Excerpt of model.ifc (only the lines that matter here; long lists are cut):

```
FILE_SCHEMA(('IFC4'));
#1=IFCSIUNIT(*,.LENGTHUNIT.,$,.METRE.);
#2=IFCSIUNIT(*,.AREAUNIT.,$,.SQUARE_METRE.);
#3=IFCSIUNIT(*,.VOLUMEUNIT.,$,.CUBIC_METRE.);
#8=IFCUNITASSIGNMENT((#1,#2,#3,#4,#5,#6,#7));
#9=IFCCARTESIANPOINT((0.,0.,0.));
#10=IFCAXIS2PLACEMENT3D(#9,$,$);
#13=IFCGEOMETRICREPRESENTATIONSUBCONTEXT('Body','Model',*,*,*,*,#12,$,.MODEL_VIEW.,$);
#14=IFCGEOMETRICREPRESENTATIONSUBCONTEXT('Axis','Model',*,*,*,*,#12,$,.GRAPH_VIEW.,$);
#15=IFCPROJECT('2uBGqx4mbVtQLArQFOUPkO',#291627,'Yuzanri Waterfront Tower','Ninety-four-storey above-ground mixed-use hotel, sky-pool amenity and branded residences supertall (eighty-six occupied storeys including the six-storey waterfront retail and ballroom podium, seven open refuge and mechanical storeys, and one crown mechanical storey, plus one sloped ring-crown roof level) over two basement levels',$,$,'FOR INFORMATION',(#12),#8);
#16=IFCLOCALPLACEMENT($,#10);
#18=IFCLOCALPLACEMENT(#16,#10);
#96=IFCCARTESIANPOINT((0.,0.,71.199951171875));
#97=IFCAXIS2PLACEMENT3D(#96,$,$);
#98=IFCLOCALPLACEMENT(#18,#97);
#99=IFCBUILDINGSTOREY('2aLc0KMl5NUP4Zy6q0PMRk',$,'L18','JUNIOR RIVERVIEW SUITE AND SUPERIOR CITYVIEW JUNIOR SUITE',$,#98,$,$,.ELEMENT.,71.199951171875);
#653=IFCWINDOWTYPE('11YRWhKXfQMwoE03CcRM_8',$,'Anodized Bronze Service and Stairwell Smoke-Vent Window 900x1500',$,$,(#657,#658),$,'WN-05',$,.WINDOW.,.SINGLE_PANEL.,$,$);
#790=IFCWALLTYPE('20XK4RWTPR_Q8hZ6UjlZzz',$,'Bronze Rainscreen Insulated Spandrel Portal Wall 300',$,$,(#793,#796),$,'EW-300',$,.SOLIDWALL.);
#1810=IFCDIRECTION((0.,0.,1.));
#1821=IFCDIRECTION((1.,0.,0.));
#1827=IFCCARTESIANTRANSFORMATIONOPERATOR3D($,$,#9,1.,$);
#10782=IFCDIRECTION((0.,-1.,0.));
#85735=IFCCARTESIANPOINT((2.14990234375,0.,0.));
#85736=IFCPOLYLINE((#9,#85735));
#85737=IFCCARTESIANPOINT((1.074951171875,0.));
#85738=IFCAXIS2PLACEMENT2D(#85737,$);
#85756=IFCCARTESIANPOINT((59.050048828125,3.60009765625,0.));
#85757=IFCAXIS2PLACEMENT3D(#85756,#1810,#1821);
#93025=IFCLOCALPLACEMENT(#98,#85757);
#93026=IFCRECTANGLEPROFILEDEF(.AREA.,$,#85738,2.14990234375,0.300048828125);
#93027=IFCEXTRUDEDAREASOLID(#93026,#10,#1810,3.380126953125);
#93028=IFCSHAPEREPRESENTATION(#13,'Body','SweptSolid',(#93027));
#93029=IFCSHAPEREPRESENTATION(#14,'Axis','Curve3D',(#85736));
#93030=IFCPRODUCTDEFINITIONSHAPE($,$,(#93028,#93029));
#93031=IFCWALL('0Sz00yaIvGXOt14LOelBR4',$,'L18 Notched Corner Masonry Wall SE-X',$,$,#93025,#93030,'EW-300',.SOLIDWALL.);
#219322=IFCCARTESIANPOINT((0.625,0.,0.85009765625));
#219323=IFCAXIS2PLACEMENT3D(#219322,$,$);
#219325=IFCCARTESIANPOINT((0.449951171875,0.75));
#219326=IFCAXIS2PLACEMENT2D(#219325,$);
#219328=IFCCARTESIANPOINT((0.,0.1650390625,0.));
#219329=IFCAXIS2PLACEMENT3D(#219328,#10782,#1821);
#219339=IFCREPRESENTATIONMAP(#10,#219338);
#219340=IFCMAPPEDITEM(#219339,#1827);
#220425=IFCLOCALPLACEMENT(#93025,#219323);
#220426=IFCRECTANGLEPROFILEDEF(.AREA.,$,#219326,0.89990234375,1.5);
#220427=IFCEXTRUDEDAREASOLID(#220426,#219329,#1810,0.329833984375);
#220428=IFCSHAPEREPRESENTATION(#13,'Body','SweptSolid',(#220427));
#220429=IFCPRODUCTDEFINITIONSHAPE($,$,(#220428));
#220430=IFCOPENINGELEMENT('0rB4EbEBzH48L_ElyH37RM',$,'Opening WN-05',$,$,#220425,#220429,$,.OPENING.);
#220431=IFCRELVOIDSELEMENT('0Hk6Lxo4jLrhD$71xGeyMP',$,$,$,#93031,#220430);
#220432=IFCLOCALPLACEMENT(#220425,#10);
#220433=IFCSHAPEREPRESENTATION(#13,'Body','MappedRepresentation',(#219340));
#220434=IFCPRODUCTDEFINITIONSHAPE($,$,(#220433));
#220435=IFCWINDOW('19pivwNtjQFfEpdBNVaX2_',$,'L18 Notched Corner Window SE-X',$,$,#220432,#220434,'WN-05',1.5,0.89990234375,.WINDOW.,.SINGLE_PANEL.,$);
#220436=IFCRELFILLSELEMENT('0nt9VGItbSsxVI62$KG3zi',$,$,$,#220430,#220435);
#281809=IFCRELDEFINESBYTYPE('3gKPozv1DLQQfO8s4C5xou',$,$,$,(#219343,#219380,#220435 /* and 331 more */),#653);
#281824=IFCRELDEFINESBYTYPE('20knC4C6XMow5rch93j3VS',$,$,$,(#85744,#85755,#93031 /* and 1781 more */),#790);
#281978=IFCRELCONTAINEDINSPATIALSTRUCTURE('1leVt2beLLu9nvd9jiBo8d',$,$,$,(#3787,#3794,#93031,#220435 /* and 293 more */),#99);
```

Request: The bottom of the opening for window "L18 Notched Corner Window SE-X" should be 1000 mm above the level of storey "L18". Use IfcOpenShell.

```python
import numpy as np
import ifcopenshell
import ifcopenshell.api.geometry
import ifcopenshell.geom
import ifcopenshell.util.element
import ifcopenshell.util.placement
import ifcopenshell.util.shape
import ifcopenshell.util.unit

model = ifcopenshell.open("model.ifc")
unit_scale = ifcopenshell.util.unit.calculate_unit_scale(model)

window = model.by_guid("19pivwNtjQFfEpdBNVaX2_")
opening = window.FillsVoids[0].RelatingOpeningElement
storey = ifcopenshell.util.element.get_container(window, ifc_class="IfcBuildingStorey")
level = ifcopenshell.util.placement.get_local_placement(storey.ObjectPlacement)[2, 3]

# The opening's origin need not be at the sill, so measure its lowest point.
shape = ifcopenshell.geom.create_shape(ifcopenshell.geom.settings(), opening)
bottom = ifcopenshell.util.shape.get_shape_bottom_elevation(shape, shape.geometry) / unit_scale
dz = level + 1.0 - bottom

shift = np.array([0.0, 0.0, dz])
# The window is placed relative to its opening, so it follows when the opening moves.
matrix = ifcopenshell.util.placement.get_local_placement(opening.ObjectPlacement)
matrix[:3, 3] += shift
ifcopenshell.api.geometry.edit_object_placement(
    model, product=opening, matrix=matrix, is_si=False, should_transform_children=True
)

print(f"moved by {dz * unit_scale:+.3f} m")

model.write("model_updated.ifc")
```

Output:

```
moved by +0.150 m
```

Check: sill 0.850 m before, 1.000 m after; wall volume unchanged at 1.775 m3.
